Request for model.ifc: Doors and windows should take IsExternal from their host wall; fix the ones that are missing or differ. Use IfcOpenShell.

First a look at what the model holds.

```python
import ifcopenshell
import ifcopenshell.util.element

model = ifcopenshell.open("model.ifc")
print(model.schema)
seen = {}
for e in model.by_type("IfcDoor") + model.by_type("IfcWindow"):
    if not e.FillsVoids:
        continue
    host = e.FillsVoids[0].RelatingOpeningElement.VoidsElements[0].RelatingBuildingElement
    own = ifcopenshell.util.element.get_pset(e, f"Pset_{e.is_a()[3:].removesuffix('StandardCase')}Common", "IsExternal")
    wall = ifcopenshell.util.element.get_pset(host, "Pset_WallCommon", "IsExternal")
    seen[e.is_a(), own, wall] = seen.get((e.is_a(), own, wall), 0) + 1
for (cls, own, wall), count in sorted(seen.items(), key=str):
    print(count, cls, "IsExternal:", own, "| host wall:", wall)
```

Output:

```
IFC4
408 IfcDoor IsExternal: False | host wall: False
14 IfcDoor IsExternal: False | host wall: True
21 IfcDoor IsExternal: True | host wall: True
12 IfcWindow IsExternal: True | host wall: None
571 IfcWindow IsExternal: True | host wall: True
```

```python
import ifcopenshell
import ifcopenshell.api.pset
import ifcopenshell.util.element

model = ifcopenshell.open("model.ifc")

count = 0
for ifc_class, pset_name in (("IfcDoor", "Pset_DoorCommon"), ("IfcWindow", "Pset_WindowCommon")):
    for e in model.by_type(ifc_class):
        if not e.FillsVoids:
            continue
        host = e.FillsVoids[0].RelatingOpeningElement.VoidsElements[0].RelatingBuildingElement
        external = ifcopenshell.util.element.get_pset(host, "Pset_WallCommon", "IsExternal")
        if external is None or ifcopenshell.util.element.get_pset(e, pset_name, "IsExternal") == external:
            continue
        pset = ifcopenshell.api.pset.add_pset(model, product=e, name=pset_name)
        ifcopenshell.api.pset.edit_pset(model, pset=pset, properties={"IsExternal": external})
        count += 1

print(count, "updated")

model.write("model_v2.ifc")
```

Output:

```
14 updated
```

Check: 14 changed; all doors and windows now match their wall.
